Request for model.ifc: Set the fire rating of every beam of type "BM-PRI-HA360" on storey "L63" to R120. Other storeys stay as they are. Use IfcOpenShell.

First a look at what the model holds.

```python
import ifcopenshell
import ifcopenshell.util.element

model = ifcopenshell.open("model.ifc")
print(model.schema)
storey = next(s for s in model.by_type("IfcBuildingStorey") if s.Name == "L63")
beams = [e for e in ifcopenshell.util.element.get_decomposition(storey) if e.is_a("IfcBeam")]
seen = {}
for e in beams:
    element_type = ifcopenshell.util.element.get_type(e)
    key = (element_type.Name if element_type != e and element_type else None, ifcopenshell.util.element.get_pset(e, "Pset_BeamCommon", "FireRating"))
    seen[key] = seen.get(key, 0) + 1
for (name, value), count in sorted(seen.items(), key=str):
    print(count, "x", name, "|", value)
```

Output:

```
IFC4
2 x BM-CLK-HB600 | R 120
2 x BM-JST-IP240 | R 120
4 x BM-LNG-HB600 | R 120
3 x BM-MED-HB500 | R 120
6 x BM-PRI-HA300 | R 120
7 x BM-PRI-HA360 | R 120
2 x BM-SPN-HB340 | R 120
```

```python
import ifcopenshell
import ifcopenshell.api.pset
import ifcopenshell.util.element

model = ifcopenshell.open("model.ifc")

storey = next(s for s in model.by_type("IfcBuildingStorey") if s.Name == "L63")
beams = [e for e in ifcopenshell.util.element.get_decomposition(storey) if e.is_a("IfcBeam")]

count = 0
for e in beams:
    element_type = ifcopenshell.util.element.get_type(e)
    if element_type in (None, e) or element_type.Name != "BM-PRI-HA360":
        continue
    found = ifcopenshell.util.element.get_pset(e, "Pset_BeamCommon", should_inherit=False)
    if found:
        pset = model.by_id(found["id"])
        if len(ifcopenshell.util.element.get_elements_by_pset(pset)) > 1:
            pset = ifcopenshell.api.pset.unshare_pset(model, products=[e], pset=pset)[0]
    else:
        pset = ifcopenshell.api.pset.add_pset(model, product=e, name="Pset_BeamCommon")
    ifcopenshell.api.pset.edit_pset(model, pset=pset, properties={"FireRating": "R120"})
    count += 1

print(count, "beams updated")

model.write("model-out.ifc")
```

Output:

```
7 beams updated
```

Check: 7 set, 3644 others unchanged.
